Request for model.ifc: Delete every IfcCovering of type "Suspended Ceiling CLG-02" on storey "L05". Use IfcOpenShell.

First a look at what the model holds.

```python
import ifcopenshell
import ifcopenshell.util.element

model = ifcopenshell.open("model.ifc")
print(model.schema)
storey = next(s for s in model.by_type("IfcBuildingStorey") if s.Name == "L05")
coverings = [e for e in ifcopenshell.util.element.get_decomposition(storey) if e.is_a("IfcCovering")]
seen = {}
for e in coverings:
    element_type = ifcopenshell.util.element.get_type(e)
    name = element_type.Name if element_type not in (None, e) else None
    seen[name] = seen.get(name, 0) + 1
for name, count in sorted(seen.items(), key=str):
    print(count, "x", name)
```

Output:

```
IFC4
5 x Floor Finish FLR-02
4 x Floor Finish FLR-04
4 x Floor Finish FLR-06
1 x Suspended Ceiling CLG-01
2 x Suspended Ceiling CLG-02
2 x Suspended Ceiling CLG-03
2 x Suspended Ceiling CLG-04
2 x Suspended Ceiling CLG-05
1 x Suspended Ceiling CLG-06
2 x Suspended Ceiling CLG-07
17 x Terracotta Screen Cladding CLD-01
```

```python
import ifcopenshell
import ifcopenshell.api.root
import ifcopenshell.util.element

model = ifcopenshell.open("model.ifc")

storey = next(s for s in model.by_type("IfcBuildingStorey") if s.Name == "L05")
coverings = [e for e in ifcopenshell.util.element.get_decomposition(storey) if e.is_a("IfcCovering")]
targets = [e for e in coverings if (t := ifcopenshell.util.element.get_type(e)) not in (None, e) and t.Name == "Suspended Ceiling CLG-02"]

for e in targets:
    ifcopenshell.api.root.remove_product(model, product=e)
print(len(targets), "removed")

model.write("model_updated.ifc")
```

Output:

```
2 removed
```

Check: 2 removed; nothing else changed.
